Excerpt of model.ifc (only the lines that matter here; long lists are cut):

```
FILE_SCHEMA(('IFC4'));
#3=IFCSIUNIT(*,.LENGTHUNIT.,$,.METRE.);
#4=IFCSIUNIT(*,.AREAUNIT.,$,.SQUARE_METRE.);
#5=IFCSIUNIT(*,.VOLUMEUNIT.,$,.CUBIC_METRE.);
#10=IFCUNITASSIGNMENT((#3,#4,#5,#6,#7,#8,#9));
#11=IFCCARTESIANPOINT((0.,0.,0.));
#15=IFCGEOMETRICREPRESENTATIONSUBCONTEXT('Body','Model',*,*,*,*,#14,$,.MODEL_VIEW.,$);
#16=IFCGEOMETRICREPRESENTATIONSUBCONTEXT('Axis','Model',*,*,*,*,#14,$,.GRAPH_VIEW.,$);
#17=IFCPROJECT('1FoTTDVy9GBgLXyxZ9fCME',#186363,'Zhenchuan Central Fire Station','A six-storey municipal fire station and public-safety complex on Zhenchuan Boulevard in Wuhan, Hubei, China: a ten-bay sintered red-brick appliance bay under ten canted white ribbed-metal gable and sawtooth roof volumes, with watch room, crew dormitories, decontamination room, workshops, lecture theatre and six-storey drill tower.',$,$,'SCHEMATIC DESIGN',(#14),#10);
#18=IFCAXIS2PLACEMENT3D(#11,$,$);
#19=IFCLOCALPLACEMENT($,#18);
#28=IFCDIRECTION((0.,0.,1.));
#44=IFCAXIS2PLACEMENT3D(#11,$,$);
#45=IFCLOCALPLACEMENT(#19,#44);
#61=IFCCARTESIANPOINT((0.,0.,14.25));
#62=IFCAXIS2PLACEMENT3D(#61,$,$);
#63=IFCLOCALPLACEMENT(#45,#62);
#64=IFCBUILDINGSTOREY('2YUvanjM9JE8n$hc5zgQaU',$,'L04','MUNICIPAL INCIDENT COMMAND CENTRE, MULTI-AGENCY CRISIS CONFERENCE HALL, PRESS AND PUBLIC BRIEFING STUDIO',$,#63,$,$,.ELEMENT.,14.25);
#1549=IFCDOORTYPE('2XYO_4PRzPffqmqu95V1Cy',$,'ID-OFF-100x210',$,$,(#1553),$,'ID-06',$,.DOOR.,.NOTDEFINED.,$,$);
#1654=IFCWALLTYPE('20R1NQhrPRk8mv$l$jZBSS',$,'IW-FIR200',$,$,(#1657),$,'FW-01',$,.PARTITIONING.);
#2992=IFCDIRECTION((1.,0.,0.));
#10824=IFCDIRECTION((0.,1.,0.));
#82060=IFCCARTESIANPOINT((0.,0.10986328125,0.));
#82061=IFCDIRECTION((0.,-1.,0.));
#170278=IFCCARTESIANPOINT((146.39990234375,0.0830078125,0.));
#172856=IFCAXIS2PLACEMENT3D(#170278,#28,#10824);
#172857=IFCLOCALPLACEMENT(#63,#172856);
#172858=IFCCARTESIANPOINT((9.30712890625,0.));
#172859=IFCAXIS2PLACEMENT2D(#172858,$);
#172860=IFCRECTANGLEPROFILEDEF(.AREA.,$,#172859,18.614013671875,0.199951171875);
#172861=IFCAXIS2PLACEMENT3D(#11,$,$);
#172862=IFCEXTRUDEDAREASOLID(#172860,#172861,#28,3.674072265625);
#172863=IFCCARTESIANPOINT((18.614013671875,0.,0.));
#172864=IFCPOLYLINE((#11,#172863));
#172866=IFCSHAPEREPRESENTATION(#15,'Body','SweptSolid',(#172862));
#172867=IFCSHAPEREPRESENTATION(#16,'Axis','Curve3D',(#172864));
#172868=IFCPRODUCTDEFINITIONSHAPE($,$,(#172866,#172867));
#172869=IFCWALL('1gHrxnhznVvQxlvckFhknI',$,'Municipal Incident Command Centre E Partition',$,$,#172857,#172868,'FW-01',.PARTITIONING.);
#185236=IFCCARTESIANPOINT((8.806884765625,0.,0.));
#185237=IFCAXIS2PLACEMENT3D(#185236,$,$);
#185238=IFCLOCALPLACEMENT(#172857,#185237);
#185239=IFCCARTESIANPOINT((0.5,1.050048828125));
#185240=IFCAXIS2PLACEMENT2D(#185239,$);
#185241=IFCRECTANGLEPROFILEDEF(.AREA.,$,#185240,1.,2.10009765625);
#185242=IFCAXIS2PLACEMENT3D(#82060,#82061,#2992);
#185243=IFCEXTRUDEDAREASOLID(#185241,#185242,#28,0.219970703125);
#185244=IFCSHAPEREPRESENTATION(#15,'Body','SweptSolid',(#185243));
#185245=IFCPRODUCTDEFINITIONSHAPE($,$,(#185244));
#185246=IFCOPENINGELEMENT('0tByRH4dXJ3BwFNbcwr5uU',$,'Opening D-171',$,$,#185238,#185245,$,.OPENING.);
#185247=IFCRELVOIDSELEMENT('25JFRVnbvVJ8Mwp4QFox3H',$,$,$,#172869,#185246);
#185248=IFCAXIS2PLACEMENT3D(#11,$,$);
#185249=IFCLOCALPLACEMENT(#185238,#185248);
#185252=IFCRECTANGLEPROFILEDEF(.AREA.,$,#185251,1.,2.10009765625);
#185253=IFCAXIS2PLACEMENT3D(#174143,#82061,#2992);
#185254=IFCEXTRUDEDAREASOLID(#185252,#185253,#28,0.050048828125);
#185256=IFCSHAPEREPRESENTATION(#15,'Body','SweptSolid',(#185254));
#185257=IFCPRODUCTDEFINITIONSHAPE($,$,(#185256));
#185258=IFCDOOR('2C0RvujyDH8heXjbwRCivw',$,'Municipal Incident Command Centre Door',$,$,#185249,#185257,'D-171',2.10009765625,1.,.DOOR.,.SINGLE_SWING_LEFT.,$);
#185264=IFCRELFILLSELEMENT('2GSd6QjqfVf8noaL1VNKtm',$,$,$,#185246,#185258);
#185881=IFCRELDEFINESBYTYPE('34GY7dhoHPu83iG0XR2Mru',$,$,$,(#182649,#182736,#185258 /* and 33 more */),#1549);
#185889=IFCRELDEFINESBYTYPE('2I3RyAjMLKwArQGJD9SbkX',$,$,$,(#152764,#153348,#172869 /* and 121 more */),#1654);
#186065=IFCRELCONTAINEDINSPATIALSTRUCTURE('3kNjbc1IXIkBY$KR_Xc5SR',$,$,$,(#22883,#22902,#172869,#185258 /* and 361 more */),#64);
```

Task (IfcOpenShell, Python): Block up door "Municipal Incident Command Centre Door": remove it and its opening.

```python
import ifcopenshell
import ifcopenshell.api.feature
import ifcopenshell.api.root
import ifcopenshell.geom
import ifcopenshell.util.shape

model = ifcopenshell.open("model.ifc")
settings = ifcopenshell.geom.settings()


def volume(element):
    """Net volume in cubic metres, openings subtracted."""
    shape = ifcopenshell.geom.create_shape(settings, element)
    return ifcopenshell.util.shape.get_volume(shape.geometry)


door = model.by_id(185258)
opening = door.FillsVoids[0].RelatingOpeningElement
wall = opening.VoidsElements[0].RelatingBuildingElement
before = volume(wall)

ifcopenshell.api.root.remove_product(model, product=door)
ifcopenshell.api.feature.remove_feature(model, feature=opening)

after = volume(wall)

print(f"wall volume {before:.3f} -> {after:.3f} m3")

model.write("model-out.ifc")
```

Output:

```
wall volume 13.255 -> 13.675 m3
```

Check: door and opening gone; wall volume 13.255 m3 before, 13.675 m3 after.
